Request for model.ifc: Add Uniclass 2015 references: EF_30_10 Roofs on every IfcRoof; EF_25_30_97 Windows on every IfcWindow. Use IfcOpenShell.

First a look at what the model holds.

```python
import ifcopenshell

model = ifcopenshell.open("model.ifc")
print(model.schema)
print("classifications:", [c.Name for c in model.by_type("IfcClassification")])
for ifc_class in ("IfcDoor", "IfcRoof", "IfcStair", "IfcWall", "IfcWindow"):
    print(ifc_class, len(model.by_type(ifc_class)))
```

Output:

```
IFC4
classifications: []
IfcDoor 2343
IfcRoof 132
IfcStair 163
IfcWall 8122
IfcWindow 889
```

```python
import ifcopenshell
import ifcopenshell.api.classification

model = ifcopenshell.open("model.ifc")

system = ifcopenshell.api.classification.add_classification(model, classification="Uniclass 2015")

codes = {
    "IfcRoof": ("EF_30_10", "Roofs"),
    "IfcWindow": ("EF_25_30_97", "Windows"),
}
for ifc_class, (code, name) in codes.items():
    products = model.by_type(ifc_class)
    ifcopenshell.api.classification.add_reference(
        model, products=products, classification=system, identification=code, name=name
    )
    print(code, len(products))

model.write("model_rev.ifc")
```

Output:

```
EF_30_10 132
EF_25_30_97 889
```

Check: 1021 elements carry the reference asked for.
